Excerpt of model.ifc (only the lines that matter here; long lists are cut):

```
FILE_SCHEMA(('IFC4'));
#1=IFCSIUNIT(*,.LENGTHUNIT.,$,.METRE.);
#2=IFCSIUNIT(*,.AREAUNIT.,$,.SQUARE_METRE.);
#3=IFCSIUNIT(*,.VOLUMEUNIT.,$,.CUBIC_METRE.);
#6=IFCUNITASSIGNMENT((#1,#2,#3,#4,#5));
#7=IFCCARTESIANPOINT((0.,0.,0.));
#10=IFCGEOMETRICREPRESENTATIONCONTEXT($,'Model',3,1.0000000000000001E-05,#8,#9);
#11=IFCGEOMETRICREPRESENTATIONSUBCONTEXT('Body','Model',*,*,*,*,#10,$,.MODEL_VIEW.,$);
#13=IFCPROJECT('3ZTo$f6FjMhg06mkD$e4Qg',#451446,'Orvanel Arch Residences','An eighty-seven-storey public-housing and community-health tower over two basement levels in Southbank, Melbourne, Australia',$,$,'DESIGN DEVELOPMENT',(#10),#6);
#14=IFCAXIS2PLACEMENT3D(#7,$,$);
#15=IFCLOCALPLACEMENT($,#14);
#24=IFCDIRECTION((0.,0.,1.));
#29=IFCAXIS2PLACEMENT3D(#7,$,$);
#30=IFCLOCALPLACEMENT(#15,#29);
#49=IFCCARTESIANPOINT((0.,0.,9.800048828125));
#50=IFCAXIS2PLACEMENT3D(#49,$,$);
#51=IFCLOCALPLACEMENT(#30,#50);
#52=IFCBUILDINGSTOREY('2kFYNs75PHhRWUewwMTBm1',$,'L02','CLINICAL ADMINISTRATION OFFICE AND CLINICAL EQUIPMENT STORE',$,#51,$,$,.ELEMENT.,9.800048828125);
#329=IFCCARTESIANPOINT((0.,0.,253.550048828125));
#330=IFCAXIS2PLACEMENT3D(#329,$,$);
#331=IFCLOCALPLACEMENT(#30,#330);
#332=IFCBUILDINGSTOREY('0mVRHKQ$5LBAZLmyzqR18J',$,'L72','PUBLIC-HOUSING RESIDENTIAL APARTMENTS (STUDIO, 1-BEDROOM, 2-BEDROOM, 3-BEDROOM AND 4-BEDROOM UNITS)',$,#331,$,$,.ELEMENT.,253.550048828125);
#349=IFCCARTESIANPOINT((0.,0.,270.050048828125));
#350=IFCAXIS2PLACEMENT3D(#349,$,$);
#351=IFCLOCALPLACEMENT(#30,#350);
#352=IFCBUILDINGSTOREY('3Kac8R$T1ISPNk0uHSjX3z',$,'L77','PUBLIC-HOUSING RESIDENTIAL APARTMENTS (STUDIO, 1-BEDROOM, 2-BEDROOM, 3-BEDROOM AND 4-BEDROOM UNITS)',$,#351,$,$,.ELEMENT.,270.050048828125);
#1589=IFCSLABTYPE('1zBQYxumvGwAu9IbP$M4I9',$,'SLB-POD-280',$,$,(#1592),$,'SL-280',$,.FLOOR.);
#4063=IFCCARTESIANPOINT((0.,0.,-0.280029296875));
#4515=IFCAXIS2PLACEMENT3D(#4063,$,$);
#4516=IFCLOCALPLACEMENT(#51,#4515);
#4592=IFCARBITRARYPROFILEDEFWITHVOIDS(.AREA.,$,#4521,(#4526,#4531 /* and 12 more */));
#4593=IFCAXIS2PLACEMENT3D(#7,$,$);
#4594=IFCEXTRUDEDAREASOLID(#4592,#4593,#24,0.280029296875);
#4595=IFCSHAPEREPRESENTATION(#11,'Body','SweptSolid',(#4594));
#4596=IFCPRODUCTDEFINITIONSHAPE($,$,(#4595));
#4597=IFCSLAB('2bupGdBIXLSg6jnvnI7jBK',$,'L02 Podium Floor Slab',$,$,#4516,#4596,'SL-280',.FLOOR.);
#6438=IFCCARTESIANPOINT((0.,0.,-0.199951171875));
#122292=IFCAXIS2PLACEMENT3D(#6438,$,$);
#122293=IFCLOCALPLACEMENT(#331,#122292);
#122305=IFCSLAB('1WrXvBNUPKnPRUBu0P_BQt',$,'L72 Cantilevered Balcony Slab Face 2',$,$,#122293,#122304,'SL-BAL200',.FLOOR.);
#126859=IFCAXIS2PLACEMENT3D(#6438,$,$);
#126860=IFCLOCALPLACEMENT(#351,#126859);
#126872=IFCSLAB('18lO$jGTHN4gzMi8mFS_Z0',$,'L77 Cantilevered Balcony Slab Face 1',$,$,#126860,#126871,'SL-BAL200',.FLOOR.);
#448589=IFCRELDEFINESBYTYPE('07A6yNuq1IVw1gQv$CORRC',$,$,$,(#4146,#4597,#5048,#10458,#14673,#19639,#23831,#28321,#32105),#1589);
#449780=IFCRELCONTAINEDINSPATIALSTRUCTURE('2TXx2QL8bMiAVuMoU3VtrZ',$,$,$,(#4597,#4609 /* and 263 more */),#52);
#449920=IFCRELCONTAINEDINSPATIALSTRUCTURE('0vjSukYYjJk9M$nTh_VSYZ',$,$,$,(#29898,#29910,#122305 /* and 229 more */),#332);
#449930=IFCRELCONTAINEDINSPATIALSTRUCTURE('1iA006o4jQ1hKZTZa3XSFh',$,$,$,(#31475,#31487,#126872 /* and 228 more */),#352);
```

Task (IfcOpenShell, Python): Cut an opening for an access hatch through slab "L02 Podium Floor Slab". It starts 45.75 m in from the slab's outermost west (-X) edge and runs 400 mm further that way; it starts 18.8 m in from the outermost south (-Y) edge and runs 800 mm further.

```python
import numpy as np
import ifcopenshell
import ifcopenshell.api.feature
import ifcopenshell.api.geometry
import ifcopenshell.api.root
import ifcopenshell.geom
import ifcopenshell.util.placement
import ifcopenshell.util.representation
import ifcopenshell.util.shape
import ifcopenshell.util.unit

model = ifcopenshell.open("model.ifc")
unit_scale = ifcopenshell.util.unit.calculate_unit_scale(model)
settings = ifcopenshell.geom.settings()


def volume(element):
    """Net volume in cubic metres, openings subtracted."""
    shape = ifcopenshell.geom.create_shape(settings, element)
    return ifcopenshell.util.shape.get_volume(shape.geometry)


slab = model.by_id(4597)
before = volume(slab)

# Extent in the slab's own axes, in metres. The edges named are its -X and -Y sides.
slab_shape = ifcopenshell.geom.create_shape(settings, slab)
vertices = ifcopenshell.util.shape.get_vertices(slab_shape.geometry)
x_min, y_min, bottom = vertices.min(axis=0)
top = vertices[:, 2].max()

opening = ifcopenshell.api.root.create_entity(model, ifc_class="IfcOpeningElement", name="Access hatch opening", predefined_type="OPENING")
context = ifcopenshell.util.representation.get_context(model, "Model", "Body", "MODEL_VIEW")
width, depth = 0.4, 0.8
outline = [(0.0, 0.0), (width, 0.0), (width, depth), (0.0, depth), (0.0, 0.0)]
# Overshoot both faces by 50 mm so the cut is clean.
shape = ifcopenshell.api.geometry.add_slab_representation(
    model, context=context, depth=top - bottom + 0.1, polyline=outline
)
ifcopenshell.api.geometry.assign_representation(model, product=opening, representation=shape)

matrix = ifcopenshell.util.placement.get_local_placement(slab.ObjectPlacement)
matrix[:, 3] = matrix @ np.append(np.array([x_min + 45.75, y_min + 18.8, bottom - 0.05]) / unit_scale, 1.0)
ifcopenshell.api.geometry.edit_object_placement(model, product=opening, matrix=matrix, is_si=False)
ifcopenshell.api.feature.add_feature(model, feature=opening, element=slab)

after = volume(slab)

print(f"slab volume {before:.3f} -> {after:.3f} m3")

model.write("model_edited.ifc")
```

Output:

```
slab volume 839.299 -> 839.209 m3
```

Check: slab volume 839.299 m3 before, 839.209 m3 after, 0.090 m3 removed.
